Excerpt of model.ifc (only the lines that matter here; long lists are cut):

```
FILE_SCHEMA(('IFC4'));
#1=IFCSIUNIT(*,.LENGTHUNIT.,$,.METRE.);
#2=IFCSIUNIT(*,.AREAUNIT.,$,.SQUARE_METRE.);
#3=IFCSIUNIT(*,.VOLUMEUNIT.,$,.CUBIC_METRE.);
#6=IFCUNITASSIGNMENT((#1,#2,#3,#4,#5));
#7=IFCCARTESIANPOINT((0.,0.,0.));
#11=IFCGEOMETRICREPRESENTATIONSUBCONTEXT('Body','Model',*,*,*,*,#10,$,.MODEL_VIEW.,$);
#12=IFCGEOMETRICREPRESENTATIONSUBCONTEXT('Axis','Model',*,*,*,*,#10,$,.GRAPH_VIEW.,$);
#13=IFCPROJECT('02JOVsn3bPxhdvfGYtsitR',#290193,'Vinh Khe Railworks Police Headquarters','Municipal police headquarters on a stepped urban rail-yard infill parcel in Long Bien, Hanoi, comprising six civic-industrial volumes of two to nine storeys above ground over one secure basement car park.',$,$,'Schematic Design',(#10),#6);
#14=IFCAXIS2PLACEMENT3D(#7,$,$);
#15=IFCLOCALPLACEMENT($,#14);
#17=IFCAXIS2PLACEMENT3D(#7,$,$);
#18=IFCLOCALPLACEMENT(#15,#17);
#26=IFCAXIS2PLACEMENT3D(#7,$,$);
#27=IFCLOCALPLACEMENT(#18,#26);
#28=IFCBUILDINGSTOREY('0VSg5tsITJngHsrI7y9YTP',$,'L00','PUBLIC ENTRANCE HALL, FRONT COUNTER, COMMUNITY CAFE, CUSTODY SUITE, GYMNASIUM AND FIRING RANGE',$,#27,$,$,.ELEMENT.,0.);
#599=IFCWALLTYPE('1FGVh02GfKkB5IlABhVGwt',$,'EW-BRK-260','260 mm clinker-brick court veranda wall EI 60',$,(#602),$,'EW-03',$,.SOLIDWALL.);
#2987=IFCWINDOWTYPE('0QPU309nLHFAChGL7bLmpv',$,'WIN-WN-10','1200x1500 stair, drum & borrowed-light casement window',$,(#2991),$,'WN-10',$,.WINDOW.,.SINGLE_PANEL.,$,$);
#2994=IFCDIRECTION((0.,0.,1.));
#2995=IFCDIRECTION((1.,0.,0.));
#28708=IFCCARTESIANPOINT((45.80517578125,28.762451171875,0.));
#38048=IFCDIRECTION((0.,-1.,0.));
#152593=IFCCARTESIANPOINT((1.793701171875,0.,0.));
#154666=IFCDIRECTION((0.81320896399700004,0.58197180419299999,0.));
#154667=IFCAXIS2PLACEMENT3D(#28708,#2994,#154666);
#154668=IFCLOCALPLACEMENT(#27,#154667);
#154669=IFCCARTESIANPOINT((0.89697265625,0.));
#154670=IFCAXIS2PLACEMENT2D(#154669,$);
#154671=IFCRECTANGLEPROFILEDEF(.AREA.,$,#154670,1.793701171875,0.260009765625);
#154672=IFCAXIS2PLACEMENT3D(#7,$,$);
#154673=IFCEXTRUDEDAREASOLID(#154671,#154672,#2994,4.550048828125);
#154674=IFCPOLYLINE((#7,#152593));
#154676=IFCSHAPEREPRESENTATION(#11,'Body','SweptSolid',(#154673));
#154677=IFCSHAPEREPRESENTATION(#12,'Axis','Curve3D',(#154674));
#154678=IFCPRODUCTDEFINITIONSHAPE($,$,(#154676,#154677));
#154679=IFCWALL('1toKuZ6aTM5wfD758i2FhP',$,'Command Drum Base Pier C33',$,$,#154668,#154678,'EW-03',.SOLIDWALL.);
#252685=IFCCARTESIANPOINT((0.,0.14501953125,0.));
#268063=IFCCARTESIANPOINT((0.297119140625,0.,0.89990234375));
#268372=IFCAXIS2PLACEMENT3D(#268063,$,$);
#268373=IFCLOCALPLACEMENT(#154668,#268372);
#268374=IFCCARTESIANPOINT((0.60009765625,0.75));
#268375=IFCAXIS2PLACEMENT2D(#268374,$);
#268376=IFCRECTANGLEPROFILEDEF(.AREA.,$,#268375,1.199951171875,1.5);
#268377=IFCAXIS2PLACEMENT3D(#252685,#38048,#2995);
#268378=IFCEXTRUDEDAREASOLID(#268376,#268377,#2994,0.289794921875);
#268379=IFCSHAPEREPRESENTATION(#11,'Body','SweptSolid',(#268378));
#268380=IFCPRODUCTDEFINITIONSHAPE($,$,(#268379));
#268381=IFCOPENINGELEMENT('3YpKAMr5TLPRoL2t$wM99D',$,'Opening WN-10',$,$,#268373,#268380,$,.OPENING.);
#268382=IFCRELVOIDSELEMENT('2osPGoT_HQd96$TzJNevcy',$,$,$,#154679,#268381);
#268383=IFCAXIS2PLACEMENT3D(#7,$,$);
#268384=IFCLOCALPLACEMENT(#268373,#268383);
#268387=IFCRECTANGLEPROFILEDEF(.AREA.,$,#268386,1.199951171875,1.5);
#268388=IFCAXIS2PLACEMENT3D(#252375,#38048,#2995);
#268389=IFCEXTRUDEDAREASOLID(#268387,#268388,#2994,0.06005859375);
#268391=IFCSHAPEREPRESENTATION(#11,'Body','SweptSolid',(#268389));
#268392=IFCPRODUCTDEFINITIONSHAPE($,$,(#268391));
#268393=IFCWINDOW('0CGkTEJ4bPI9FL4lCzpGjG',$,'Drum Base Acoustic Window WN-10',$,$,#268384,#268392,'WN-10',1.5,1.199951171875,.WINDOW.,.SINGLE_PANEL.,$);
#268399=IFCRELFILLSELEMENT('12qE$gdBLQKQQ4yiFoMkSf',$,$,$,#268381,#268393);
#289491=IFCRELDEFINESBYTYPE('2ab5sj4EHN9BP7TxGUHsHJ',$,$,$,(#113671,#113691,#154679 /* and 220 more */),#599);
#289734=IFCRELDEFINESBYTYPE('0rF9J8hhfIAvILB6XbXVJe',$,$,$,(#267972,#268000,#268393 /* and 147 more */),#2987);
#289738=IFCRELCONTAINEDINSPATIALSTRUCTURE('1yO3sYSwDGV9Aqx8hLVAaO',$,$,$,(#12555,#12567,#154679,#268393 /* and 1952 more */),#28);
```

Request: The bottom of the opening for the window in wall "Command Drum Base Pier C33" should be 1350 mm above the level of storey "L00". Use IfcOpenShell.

```python
import numpy as np
import ifcopenshell
import ifcopenshell.api.geometry
import ifcopenshell.geom
import ifcopenshell.util.element
import ifcopenshell.util.placement
import ifcopenshell.util.shape
import ifcopenshell.util.unit

model = ifcopenshell.open("model.ifc")
unit_scale = ifcopenshell.util.unit.calculate_unit_scale(model)

window = model.by_guid("0CGkTEJ4bPI9FL4lCzpGjG")
opening = window.FillsVoids[0].RelatingOpeningElement
storey = ifcopenshell.util.element.get_container(window, ifc_class="IfcBuildingStorey")
level = ifcopenshell.util.placement.get_local_placement(storey.ObjectPlacement)[2, 3]

# The opening's origin need not be at the sill, so measure its lowest point.
shape = ifcopenshell.geom.create_shape(ifcopenshell.geom.settings(), opening)
bottom = ifcopenshell.util.shape.get_shape_bottom_elevation(shape, shape.geometry) / unit_scale
dz = level + 1.35 / unit_scale - bottom

shift = np.array([0.0, 0.0, dz])
# The window is placed relative to its opening, so it follows when the opening moves.
matrix = ifcopenshell.util.placement.get_local_placement(opening.ObjectPlacement)
matrix[:3, 3] += shift
ifcopenshell.api.geometry.edit_object_placement(
    model, product=opening, matrix=matrix, is_si=False, should_transform_children=True
)

print(f"moved by {dz * unit_scale:+.3f} m")

model.write("model-out.ifc")
```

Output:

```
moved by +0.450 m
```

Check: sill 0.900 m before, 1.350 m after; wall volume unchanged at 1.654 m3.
